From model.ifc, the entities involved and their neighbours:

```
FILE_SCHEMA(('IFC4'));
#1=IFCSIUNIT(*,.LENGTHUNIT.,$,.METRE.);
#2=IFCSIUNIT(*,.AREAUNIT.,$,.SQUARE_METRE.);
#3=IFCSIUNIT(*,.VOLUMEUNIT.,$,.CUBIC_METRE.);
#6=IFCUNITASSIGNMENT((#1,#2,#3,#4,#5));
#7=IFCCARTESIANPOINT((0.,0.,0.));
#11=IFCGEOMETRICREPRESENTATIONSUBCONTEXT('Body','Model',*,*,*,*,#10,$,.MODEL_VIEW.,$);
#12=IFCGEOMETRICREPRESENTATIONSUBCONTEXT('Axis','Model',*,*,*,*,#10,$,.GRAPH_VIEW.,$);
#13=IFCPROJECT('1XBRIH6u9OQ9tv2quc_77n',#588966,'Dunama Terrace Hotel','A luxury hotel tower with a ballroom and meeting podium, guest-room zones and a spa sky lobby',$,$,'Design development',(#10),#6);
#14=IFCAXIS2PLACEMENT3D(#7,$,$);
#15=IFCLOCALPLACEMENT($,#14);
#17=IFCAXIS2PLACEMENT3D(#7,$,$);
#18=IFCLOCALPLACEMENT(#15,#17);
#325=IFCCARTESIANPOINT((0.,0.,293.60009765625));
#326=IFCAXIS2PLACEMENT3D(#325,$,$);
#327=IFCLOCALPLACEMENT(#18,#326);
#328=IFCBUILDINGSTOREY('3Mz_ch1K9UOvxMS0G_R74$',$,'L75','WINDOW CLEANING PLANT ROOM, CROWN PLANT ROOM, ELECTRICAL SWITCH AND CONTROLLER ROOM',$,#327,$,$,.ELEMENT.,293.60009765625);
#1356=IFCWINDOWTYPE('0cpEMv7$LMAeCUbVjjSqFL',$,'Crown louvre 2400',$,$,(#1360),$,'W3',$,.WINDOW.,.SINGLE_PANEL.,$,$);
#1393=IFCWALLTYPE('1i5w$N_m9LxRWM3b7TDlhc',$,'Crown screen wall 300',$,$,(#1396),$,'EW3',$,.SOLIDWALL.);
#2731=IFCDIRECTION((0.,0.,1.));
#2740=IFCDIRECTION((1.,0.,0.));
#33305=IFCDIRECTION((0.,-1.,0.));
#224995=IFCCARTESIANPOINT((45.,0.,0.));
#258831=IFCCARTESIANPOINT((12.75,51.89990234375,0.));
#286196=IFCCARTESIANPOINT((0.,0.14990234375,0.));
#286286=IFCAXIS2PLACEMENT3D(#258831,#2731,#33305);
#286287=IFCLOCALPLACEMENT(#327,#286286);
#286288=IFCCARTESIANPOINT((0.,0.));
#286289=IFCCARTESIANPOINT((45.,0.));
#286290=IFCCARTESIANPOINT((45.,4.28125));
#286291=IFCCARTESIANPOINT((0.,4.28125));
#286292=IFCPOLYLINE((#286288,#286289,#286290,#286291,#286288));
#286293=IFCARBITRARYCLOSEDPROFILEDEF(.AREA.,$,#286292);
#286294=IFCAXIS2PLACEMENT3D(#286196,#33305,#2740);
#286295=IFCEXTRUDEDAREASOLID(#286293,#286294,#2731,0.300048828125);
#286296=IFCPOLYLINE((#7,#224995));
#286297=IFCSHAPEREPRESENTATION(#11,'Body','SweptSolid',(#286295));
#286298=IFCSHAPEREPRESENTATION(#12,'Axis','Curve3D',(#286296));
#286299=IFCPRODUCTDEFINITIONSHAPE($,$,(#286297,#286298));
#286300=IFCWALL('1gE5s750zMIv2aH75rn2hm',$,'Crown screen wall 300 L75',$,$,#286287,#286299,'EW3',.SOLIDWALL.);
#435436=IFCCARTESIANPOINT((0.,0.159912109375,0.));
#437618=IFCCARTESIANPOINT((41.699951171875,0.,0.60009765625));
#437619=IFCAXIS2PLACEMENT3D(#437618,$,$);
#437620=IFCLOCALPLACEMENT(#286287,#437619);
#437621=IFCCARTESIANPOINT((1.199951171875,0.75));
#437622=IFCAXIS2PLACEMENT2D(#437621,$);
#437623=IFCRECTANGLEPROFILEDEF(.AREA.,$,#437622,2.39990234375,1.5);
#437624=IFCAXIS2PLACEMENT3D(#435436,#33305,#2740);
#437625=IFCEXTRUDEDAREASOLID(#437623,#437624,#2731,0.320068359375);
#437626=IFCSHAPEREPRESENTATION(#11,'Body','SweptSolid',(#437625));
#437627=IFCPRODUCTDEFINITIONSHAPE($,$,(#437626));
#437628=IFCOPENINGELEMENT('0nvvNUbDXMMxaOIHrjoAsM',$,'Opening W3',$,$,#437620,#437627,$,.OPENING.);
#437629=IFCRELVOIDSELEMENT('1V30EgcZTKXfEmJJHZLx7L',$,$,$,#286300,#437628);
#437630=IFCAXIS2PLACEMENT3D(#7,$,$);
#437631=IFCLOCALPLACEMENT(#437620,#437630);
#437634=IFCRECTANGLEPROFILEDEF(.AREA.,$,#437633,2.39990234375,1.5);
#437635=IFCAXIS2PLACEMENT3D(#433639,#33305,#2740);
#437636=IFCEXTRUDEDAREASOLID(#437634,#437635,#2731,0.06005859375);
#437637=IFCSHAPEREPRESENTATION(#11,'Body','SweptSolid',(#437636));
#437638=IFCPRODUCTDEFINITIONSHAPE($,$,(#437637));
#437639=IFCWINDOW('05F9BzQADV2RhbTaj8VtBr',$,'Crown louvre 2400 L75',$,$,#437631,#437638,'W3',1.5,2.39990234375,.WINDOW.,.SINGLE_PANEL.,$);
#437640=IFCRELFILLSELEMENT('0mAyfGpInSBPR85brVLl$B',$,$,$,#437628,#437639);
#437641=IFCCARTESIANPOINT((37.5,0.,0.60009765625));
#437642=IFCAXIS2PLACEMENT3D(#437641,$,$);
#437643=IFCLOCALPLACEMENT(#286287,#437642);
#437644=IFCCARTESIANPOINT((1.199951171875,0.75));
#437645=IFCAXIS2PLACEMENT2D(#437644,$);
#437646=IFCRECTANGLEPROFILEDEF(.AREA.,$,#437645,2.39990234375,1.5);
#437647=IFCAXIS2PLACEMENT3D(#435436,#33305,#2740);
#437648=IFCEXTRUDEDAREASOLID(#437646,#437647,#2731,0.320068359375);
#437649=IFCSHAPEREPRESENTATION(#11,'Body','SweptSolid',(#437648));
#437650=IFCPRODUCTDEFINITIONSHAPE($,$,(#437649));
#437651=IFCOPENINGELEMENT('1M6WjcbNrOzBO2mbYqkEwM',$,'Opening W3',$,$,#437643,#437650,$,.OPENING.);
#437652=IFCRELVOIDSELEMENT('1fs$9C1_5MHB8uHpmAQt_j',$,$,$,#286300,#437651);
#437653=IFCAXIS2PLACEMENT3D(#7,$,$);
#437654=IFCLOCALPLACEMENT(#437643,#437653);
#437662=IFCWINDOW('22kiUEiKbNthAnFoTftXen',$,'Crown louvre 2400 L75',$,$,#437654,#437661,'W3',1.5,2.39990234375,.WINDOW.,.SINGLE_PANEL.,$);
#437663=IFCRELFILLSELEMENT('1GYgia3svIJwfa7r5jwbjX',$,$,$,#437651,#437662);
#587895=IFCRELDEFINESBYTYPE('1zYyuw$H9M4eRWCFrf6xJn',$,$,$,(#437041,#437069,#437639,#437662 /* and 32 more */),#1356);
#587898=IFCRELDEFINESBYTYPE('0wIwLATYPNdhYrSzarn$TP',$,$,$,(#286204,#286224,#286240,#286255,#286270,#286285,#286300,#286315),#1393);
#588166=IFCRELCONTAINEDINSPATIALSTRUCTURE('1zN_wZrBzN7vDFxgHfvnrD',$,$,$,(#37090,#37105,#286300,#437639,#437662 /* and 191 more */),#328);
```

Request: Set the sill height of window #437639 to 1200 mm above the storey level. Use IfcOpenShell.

```python
import numpy as np
import ifcopenshell
import ifcopenshell.api.geometry
import ifcopenshell.geom
import ifcopenshell.util.element
import ifcopenshell.util.placement
import ifcopenshell.util.shape
import ifcopenshell.util.unit

model = ifcopenshell.open("model.ifc")
unit_scale = ifcopenshell.util.unit.calculate_unit_scale(model)

window = model.by_guid("05F9BzQADV2RhbTaj8VtBr")
opening = window.FillsVoids[0].RelatingOpeningElement
storey = ifcopenshell.util.element.get_container(window, ifc_class="IfcBuildingStorey")
level = ifcopenshell.util.placement.get_local_placement(storey.ObjectPlacement)[2, 3]

# The opening's origin need not be at the sill, so measure its lowest point.
shape = ifcopenshell.geom.create_shape(ifcopenshell.geom.settings(), opening)
bottom = ifcopenshell.util.shape.get_shape_bottom_elevation(shape, shape.geometry) / unit_scale
dz = level + 1.2 / unit_scale - bottom

shift = np.array([0.0, 0.0, dz])
# The window is placed relative to its opening, so it follows when the opening moves.
matrix = ifcopenshell.util.placement.get_local_placement(opening.ObjectPlacement)
matrix[:3, 3] += shift
ifcopenshell.api.geometry.edit_object_placement(
    model, product=opening, matrix=matrix, is_si=False, should_transform_children=True
)

print(f"moved by {dz * unit_scale:+.3f} m")

model.write("model-out.ifc")
```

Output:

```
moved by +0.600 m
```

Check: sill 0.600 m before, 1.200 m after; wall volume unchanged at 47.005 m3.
